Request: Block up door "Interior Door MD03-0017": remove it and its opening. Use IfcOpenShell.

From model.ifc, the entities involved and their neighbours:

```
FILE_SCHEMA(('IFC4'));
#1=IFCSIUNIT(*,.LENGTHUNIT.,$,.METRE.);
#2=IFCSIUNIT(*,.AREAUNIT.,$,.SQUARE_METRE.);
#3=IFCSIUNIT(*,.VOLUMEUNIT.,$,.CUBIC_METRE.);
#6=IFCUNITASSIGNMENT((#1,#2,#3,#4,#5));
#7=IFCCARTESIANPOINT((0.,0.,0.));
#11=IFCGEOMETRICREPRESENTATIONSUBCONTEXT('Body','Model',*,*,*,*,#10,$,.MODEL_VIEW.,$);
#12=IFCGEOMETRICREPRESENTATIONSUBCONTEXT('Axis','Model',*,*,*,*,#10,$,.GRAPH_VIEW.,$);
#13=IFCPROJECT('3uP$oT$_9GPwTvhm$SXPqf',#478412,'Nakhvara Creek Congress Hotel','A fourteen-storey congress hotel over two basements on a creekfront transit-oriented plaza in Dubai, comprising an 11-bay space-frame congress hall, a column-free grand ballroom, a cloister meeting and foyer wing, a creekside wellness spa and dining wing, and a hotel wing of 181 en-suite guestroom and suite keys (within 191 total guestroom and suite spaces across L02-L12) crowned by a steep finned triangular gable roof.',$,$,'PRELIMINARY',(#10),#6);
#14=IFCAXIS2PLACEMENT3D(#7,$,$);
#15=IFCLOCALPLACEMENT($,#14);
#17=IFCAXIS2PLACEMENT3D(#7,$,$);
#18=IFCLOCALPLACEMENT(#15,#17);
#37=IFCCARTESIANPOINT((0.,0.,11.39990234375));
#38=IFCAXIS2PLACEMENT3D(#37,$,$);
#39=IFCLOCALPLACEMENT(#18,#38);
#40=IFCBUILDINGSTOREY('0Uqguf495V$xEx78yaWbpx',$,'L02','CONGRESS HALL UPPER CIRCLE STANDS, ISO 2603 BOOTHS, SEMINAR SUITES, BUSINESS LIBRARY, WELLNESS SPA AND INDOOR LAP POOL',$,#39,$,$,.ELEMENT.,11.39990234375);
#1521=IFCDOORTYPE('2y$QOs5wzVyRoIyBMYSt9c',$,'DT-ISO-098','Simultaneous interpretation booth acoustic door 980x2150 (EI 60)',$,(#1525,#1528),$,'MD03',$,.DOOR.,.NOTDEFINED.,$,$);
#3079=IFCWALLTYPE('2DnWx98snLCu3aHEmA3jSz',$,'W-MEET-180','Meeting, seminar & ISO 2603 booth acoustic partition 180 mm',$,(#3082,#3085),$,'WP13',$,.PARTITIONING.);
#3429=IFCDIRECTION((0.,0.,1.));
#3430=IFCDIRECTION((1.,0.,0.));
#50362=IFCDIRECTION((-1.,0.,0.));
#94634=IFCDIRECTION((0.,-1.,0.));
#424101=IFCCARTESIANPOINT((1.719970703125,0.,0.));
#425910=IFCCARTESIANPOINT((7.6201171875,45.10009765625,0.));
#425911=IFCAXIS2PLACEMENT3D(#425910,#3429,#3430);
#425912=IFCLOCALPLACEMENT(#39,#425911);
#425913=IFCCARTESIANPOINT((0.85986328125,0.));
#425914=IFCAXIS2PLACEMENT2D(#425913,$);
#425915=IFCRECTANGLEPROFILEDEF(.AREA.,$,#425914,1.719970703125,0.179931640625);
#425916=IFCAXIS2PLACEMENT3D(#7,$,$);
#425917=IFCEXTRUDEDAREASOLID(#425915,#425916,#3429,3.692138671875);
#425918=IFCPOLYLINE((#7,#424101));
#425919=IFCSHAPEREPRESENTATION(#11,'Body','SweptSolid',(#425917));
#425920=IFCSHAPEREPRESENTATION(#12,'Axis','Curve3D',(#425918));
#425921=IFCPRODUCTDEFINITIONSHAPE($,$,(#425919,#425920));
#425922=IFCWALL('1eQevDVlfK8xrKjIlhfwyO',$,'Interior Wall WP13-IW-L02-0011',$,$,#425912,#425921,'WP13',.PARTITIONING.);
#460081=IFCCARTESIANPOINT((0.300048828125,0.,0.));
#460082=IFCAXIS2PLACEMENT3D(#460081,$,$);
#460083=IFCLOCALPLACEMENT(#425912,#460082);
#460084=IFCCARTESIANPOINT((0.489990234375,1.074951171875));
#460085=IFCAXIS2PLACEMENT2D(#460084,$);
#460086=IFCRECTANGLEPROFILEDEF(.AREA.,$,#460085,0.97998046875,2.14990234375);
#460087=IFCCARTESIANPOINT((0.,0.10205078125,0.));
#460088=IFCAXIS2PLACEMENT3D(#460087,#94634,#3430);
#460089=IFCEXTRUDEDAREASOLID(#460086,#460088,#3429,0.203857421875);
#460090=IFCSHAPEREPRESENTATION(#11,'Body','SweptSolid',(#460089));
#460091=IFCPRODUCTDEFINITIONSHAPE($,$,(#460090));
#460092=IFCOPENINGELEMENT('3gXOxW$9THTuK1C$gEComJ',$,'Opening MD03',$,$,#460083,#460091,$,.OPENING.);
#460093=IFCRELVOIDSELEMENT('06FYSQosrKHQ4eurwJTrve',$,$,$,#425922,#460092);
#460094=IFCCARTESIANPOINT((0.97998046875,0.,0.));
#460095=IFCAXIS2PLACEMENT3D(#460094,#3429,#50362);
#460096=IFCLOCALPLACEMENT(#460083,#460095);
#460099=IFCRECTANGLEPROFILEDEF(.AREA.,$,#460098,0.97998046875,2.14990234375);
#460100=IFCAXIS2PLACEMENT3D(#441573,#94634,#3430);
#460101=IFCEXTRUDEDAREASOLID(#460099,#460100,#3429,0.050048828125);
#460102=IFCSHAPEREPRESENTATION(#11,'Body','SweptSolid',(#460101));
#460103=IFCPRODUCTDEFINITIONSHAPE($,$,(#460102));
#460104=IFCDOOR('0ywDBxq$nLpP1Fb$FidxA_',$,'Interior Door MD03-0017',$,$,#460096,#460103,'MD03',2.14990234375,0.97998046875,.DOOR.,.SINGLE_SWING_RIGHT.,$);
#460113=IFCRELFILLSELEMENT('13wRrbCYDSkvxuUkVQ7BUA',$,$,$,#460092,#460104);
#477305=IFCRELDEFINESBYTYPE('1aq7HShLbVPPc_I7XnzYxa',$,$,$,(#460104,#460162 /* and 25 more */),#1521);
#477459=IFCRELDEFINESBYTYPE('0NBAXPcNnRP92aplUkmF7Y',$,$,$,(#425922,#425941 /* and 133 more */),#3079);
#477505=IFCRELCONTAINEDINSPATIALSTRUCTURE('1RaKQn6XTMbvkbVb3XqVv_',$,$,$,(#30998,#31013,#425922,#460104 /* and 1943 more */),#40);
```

```python
import ifcopenshell
import ifcopenshell.api.feature
import ifcopenshell.api.root
import ifcopenshell.geom
import ifcopenshell.util.shape

model = ifcopenshell.open("model.ifc")
settings = ifcopenshell.geom.settings()


def volume(element):
    """Net volume in cubic metres, openings subtracted."""
    shape = ifcopenshell.geom.create_shape(settings, element)
    return ifcopenshell.util.shape.get_volume(shape.geometry)


door = model.by_guid("0ywDBxq$nLpP1Fb$FidxA_")
opening = door.FillsVoids[0].RelatingOpeningElement
wall = opening.VoidsElements[0].RelatingBuildingElement
before = volume(wall)

ifcopenshell.api.root.remove_product(model, product=door)
ifcopenshell.api.feature.remove_feature(model, feature=opening)

after = volume(wall)

print(f"wall volume {before:.3f} -> {after:.3f} m3")

model.write("model_updated.ifc")
```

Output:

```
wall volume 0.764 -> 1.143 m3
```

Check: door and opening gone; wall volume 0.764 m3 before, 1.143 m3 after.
